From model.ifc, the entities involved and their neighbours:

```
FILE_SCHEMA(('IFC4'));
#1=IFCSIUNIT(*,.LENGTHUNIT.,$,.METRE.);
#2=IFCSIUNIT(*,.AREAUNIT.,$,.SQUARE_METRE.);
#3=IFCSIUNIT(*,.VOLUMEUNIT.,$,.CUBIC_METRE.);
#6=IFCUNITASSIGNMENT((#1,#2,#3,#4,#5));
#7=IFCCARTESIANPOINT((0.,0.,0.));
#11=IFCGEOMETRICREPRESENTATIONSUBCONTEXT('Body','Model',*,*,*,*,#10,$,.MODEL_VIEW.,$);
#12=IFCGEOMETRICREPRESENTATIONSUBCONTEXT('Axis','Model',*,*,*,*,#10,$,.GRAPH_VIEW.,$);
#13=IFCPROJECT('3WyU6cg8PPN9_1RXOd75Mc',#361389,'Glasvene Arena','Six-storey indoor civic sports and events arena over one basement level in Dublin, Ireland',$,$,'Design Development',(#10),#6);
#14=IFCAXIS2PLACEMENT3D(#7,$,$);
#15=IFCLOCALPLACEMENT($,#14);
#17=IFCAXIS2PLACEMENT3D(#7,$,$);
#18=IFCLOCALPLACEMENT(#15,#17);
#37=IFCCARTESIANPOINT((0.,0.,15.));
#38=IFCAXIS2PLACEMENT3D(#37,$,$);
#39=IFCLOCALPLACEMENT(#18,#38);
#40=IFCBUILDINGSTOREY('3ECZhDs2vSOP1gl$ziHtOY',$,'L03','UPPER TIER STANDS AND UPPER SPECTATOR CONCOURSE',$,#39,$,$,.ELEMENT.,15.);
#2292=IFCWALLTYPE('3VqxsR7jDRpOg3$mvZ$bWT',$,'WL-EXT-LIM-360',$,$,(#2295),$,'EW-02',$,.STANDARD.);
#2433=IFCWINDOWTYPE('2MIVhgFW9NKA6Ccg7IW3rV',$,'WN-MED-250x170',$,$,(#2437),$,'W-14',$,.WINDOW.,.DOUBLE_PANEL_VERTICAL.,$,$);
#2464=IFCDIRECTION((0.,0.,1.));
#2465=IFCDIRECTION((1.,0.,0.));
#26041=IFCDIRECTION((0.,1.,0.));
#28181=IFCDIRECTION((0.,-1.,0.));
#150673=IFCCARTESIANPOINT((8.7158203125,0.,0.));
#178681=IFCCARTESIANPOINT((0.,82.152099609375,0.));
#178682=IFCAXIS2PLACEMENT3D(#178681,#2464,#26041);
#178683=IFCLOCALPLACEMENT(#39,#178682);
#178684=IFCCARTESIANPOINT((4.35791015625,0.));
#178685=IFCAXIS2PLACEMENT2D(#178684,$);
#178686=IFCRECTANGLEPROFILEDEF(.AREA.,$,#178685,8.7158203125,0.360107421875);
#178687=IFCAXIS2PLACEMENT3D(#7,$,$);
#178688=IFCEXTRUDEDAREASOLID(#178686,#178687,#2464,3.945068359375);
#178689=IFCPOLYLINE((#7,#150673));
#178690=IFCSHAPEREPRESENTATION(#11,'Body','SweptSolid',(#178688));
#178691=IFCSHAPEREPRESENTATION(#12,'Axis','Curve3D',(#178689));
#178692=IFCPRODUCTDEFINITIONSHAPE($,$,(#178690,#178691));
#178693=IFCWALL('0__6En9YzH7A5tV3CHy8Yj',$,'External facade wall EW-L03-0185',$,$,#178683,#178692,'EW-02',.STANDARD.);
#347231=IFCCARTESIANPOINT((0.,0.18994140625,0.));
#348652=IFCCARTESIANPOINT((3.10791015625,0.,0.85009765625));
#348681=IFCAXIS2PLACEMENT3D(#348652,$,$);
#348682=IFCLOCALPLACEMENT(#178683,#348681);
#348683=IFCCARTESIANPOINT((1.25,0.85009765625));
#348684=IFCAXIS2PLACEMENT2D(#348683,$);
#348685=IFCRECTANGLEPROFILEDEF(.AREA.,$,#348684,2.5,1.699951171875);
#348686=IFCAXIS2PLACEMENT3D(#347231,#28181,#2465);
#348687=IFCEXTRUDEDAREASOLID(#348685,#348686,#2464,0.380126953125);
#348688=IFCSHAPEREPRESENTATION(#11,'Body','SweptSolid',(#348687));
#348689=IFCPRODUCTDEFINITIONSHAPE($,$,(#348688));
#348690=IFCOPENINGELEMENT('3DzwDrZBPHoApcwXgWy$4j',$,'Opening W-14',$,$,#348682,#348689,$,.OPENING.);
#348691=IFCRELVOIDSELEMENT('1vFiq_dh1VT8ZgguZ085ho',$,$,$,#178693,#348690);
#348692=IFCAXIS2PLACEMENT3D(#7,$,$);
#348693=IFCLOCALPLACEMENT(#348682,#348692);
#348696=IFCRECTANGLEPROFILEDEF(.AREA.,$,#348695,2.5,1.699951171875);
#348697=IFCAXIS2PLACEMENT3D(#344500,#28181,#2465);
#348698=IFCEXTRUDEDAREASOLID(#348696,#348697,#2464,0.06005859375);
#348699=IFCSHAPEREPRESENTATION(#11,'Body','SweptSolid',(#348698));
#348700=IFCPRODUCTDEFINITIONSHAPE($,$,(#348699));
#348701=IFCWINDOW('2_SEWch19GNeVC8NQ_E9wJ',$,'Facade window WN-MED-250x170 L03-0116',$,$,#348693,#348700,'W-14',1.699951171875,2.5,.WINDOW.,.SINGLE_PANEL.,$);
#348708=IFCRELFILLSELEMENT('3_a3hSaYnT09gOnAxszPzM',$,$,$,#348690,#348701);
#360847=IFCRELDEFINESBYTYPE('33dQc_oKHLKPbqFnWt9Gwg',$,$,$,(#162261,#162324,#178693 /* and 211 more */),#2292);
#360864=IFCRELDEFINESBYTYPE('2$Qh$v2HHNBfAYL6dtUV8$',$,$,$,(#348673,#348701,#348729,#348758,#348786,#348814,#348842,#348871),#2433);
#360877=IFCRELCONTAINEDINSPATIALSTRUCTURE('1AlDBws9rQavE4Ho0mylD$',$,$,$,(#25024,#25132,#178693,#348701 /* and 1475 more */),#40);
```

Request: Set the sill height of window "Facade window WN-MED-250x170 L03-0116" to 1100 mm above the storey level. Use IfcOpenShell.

```python
import numpy as np
import ifcopenshell
import ifcopenshell.api.geometry
import ifcopenshell.geom
import ifcopenshell.util.element
import ifcopenshell.util.placement
import ifcopenshell.util.shape
import ifcopenshell.util.unit

model = ifcopenshell.open("model.ifc")
unit_scale = ifcopenshell.util.unit.calculate_unit_scale(model)

window = model.by_id(348701)
opening = window.FillsVoids[0].RelatingOpeningElement
storey = ifcopenshell.util.element.get_container(window, ifc_class="IfcBuildingStorey")
level = ifcopenshell.util.placement.get_local_placement(storey.ObjectPlacement)[2, 3]

# The opening's origin need not be at the sill, so measure its lowest point.
shape = ifcopenshell.geom.create_shape(ifcopenshell.geom.settings(), opening)
bottom = ifcopenshell.util.shape.get_shape_bottom_elevation(shape, shape.geometry) / unit_scale
dz = level + 1.1 - bottom

shift = np.array([0.0, 0.0, dz])
# The window is placed relative to its opening, so it follows when the opening moves.
matrix = ifcopenshell.util.placement.get_local_placement(opening.ObjectPlacement)
matrix[:3, 3] += shift
ifcopenshell.api.geometry.edit_object_placement(
    model, product=opening, matrix=matrix, is_si=False, should_transform_children=True
)

print(f"moved by {dz * unit_scale:+.3f} m")

model.write("model_edited.ifc")
```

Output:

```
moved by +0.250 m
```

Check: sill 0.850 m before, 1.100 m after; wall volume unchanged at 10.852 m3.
